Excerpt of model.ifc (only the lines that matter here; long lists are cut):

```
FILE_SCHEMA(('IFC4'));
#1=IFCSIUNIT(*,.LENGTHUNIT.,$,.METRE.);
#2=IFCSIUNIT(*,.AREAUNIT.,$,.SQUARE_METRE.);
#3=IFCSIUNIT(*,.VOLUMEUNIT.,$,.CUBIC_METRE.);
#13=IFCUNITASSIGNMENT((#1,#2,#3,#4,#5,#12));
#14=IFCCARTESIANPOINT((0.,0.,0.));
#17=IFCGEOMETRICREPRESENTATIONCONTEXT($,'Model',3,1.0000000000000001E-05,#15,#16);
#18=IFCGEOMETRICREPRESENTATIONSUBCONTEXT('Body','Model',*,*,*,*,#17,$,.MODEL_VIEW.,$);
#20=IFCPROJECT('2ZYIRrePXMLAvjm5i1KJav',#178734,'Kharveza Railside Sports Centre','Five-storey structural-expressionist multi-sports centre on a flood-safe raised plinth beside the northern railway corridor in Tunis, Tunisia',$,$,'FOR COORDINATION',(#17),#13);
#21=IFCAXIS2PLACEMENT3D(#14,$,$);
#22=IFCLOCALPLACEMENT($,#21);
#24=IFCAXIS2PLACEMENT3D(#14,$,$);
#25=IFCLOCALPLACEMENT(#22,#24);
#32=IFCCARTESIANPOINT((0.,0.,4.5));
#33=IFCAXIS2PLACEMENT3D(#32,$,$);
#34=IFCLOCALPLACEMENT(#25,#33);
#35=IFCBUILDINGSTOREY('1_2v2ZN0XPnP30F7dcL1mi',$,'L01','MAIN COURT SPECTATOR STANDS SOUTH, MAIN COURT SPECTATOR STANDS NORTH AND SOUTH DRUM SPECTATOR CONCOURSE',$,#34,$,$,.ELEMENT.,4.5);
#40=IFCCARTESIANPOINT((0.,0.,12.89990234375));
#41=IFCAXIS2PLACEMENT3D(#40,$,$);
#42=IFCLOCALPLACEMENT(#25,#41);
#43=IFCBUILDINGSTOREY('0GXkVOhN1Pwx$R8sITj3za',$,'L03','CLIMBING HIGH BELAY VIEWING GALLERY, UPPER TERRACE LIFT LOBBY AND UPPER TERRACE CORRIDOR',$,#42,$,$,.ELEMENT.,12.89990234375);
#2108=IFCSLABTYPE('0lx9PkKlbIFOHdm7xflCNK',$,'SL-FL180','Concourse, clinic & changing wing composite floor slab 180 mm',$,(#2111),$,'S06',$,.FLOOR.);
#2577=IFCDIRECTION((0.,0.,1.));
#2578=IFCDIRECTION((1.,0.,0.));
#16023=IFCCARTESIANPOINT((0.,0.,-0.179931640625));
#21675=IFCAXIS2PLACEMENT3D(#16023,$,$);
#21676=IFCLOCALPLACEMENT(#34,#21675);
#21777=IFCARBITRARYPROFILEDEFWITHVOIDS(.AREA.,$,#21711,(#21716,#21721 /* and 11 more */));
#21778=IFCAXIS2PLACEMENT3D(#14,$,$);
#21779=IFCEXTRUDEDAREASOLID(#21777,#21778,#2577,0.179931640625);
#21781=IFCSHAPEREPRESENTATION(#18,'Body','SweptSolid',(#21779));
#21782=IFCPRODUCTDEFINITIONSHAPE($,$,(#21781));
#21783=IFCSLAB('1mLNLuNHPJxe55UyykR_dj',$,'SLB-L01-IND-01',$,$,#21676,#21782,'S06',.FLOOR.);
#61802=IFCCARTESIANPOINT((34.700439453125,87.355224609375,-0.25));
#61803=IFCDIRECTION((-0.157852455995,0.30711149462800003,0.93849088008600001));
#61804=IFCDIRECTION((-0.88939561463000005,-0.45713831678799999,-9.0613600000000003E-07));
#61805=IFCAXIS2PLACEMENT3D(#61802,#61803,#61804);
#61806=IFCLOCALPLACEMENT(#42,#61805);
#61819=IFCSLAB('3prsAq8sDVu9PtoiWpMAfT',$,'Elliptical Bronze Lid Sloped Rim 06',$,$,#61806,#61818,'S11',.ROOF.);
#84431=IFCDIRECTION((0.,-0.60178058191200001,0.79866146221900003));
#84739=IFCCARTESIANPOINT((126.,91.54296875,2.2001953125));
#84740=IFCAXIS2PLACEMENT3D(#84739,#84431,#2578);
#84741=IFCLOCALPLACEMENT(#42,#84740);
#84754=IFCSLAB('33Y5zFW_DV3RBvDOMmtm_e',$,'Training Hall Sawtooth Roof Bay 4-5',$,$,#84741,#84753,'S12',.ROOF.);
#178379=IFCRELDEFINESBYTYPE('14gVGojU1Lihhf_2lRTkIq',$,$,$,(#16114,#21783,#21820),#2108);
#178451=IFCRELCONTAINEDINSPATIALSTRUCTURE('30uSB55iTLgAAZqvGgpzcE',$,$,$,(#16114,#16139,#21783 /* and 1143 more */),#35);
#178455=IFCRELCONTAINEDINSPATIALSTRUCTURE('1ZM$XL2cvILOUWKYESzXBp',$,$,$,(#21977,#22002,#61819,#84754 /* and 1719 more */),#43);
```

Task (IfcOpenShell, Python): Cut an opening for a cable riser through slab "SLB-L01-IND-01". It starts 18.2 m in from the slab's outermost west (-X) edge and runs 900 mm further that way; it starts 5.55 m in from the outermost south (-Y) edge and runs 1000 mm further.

```python
import numpy as np
import ifcopenshell
import ifcopenshell.api.feature
import ifcopenshell.api.geometry
import ifcopenshell.api.root
import ifcopenshell.geom
import ifcopenshell.util.placement
import ifcopenshell.util.representation
import ifcopenshell.util.shape
import ifcopenshell.util.unit

model = ifcopenshell.open("model.ifc")
unit_scale = ifcopenshell.util.unit.calculate_unit_scale(model)
settings = ifcopenshell.geom.settings()


def volume(element):
    """Net volume in cubic metres, openings subtracted."""
    shape = ifcopenshell.geom.create_shape(settings, element)
    return ifcopenshell.util.shape.get_volume(shape.geometry)


slab = model.by_guid("1mLNLuNHPJxe55UyykR_dj")
before = volume(slab)

# Extent in the slab's own axes, in metres. The edges named are its -X and -Y sides.
slab_shape = ifcopenshell.geom.create_shape(settings, slab)
vertices = ifcopenshell.util.shape.get_vertices(slab_shape.geometry)
x_min, y_min, bottom = vertices.min(axis=0)
top = vertices[:, 2].max()

opening = ifcopenshell.api.root.create_entity(model, ifc_class="IfcOpeningElement", name="Cable riser opening", predefined_type="OPENING")
context = ifcopenshell.util.representation.get_context(model, "Model", "Body", "MODEL_VIEW")
width, depth = 0.9, 1
outline = [(0.0, 0.0), (width, 0.0), (width, depth), (0.0, depth), (0.0, 0.0)]
# Overshoot both faces by 50 mm so the cut is clean.
shape = ifcopenshell.api.geometry.add_slab_representation(
    model, context=context, depth=top - bottom + 0.1, polyline=outline
)
ifcopenshell.api.geometry.assign_representation(model, product=opening, representation=shape)

matrix = ifcopenshell.util.placement.get_local_placement(slab.ObjectPlacement)
matrix[:, 3] = matrix @ np.append(np.array([x_min + 18.2, y_min + 5.55, bottom - 0.05]) / unit_scale, 1.0)
ifcopenshell.api.geometry.edit_object_placement(model, product=opening, matrix=matrix, is_si=False)
ifcopenshell.api.feature.add_feature(model, feature=opening, element=slab)

after = volume(slab)

print(f"slab volume {before:.3f} -> {after:.3f} m3")

model.write("model-out.ifc")
```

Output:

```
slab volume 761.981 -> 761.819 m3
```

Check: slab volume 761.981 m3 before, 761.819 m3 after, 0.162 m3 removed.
